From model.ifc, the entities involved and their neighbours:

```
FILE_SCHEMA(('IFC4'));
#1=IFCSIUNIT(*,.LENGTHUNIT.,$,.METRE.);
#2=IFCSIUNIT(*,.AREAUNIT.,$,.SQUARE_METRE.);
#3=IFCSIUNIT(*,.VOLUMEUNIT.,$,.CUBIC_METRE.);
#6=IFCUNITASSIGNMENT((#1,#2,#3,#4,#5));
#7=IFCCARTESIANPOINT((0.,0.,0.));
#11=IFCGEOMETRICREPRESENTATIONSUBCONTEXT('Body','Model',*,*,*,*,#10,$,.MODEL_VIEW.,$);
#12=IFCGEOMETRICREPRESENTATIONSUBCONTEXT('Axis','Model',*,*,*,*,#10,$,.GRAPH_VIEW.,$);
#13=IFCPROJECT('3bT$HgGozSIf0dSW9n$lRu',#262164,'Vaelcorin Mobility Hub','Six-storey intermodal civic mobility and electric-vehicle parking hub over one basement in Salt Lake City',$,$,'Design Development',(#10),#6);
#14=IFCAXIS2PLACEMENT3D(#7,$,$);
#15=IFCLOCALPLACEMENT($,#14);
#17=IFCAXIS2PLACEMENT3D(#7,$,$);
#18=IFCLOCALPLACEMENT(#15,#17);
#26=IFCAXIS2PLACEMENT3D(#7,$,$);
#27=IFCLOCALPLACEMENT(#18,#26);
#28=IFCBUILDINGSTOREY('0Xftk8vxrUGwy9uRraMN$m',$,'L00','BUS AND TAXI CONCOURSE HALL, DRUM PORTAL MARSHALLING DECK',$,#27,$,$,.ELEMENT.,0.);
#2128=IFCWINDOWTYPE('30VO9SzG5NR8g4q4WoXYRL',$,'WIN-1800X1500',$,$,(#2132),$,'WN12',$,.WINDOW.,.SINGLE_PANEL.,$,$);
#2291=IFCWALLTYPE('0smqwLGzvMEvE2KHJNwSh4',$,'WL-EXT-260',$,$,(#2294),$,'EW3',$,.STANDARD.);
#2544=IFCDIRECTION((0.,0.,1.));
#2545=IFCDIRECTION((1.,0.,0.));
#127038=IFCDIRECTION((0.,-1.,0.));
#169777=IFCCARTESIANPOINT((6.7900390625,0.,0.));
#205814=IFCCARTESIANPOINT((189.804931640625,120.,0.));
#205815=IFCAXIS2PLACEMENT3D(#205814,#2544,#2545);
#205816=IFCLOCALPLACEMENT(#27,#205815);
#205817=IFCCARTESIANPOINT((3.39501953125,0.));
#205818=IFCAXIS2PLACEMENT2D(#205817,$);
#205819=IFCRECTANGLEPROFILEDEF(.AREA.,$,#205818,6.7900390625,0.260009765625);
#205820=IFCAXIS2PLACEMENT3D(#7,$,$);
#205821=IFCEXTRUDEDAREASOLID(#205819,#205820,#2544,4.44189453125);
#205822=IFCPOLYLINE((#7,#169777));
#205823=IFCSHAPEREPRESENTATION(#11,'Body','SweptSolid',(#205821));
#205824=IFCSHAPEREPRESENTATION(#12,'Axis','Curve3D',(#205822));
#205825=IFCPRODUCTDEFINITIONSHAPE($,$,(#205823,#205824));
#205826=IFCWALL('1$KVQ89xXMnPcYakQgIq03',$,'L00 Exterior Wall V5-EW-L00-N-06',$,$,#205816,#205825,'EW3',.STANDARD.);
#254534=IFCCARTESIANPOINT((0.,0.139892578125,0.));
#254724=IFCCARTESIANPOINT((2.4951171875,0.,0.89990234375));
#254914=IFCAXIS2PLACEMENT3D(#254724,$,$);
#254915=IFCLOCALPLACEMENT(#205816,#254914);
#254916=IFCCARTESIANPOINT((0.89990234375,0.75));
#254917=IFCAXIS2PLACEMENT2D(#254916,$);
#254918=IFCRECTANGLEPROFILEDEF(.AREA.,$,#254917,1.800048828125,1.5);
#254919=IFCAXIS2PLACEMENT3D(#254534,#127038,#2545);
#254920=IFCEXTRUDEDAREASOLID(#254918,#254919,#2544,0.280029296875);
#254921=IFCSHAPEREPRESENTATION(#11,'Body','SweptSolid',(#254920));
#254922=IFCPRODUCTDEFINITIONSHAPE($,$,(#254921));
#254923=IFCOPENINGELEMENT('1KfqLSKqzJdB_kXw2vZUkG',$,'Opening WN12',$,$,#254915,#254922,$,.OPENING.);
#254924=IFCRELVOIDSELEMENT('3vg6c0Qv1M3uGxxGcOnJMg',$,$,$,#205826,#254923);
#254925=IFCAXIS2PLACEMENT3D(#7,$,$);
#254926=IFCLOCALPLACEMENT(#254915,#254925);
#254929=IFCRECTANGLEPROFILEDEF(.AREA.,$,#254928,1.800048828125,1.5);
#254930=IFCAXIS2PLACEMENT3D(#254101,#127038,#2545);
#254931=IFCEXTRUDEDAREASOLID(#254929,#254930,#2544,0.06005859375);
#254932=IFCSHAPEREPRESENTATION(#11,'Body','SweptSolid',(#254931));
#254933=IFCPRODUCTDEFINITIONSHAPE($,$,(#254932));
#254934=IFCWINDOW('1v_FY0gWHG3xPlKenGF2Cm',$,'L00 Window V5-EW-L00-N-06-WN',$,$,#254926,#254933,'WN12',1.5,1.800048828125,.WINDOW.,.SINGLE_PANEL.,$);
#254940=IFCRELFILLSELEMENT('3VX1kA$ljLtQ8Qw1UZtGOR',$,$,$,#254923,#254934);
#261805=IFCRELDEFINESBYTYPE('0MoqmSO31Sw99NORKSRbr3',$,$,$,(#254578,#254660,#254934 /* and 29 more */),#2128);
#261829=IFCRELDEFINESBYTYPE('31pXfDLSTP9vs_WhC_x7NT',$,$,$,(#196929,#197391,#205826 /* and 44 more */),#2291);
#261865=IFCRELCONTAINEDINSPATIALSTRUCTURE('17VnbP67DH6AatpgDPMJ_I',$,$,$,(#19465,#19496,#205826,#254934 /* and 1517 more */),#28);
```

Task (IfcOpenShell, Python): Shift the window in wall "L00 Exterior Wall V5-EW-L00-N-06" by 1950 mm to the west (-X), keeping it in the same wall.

```python
import ifcopenshell
import ifcopenshell.api.geometry
import ifcopenshell.util.placement

model = ifcopenshell.open("model.ifc")

window = model.by_guid("1v_FY0gWHG3xPlKenGF2Cm")
opening = window.FillsVoids[0].RelatingOpeningElement
wall = opening.VoidsElements[0].RelatingBuildingElement

wall_matrix = ifcopenshell.util.placement.get_local_placement(wall.ObjectPlacement)
shift = wall_matrix[:3, 0] * -1.95
before = ifcopenshell.util.placement.get_local_placement(window.ObjectPlacement)[:3, 3].copy()

# The window is placed relative to its opening, so it follows when the opening moves.
matrix = ifcopenshell.util.placement.get_local_placement(opening.ObjectPlacement)
matrix[:3, 3] += shift
ifcopenshell.api.geometry.edit_object_placement(
    model, product=opening, matrix=matrix, is_si=False, should_transform_children=True
)

after = ifcopenshell.util.placement.get_local_placement(window.ObjectPlacement)[:3, 3]
print("window moved by", (after - before).round(3) + 0.0)

model.write("model_rev.ifc")
```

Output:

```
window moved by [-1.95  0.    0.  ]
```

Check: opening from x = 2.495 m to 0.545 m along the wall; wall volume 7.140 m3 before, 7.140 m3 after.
